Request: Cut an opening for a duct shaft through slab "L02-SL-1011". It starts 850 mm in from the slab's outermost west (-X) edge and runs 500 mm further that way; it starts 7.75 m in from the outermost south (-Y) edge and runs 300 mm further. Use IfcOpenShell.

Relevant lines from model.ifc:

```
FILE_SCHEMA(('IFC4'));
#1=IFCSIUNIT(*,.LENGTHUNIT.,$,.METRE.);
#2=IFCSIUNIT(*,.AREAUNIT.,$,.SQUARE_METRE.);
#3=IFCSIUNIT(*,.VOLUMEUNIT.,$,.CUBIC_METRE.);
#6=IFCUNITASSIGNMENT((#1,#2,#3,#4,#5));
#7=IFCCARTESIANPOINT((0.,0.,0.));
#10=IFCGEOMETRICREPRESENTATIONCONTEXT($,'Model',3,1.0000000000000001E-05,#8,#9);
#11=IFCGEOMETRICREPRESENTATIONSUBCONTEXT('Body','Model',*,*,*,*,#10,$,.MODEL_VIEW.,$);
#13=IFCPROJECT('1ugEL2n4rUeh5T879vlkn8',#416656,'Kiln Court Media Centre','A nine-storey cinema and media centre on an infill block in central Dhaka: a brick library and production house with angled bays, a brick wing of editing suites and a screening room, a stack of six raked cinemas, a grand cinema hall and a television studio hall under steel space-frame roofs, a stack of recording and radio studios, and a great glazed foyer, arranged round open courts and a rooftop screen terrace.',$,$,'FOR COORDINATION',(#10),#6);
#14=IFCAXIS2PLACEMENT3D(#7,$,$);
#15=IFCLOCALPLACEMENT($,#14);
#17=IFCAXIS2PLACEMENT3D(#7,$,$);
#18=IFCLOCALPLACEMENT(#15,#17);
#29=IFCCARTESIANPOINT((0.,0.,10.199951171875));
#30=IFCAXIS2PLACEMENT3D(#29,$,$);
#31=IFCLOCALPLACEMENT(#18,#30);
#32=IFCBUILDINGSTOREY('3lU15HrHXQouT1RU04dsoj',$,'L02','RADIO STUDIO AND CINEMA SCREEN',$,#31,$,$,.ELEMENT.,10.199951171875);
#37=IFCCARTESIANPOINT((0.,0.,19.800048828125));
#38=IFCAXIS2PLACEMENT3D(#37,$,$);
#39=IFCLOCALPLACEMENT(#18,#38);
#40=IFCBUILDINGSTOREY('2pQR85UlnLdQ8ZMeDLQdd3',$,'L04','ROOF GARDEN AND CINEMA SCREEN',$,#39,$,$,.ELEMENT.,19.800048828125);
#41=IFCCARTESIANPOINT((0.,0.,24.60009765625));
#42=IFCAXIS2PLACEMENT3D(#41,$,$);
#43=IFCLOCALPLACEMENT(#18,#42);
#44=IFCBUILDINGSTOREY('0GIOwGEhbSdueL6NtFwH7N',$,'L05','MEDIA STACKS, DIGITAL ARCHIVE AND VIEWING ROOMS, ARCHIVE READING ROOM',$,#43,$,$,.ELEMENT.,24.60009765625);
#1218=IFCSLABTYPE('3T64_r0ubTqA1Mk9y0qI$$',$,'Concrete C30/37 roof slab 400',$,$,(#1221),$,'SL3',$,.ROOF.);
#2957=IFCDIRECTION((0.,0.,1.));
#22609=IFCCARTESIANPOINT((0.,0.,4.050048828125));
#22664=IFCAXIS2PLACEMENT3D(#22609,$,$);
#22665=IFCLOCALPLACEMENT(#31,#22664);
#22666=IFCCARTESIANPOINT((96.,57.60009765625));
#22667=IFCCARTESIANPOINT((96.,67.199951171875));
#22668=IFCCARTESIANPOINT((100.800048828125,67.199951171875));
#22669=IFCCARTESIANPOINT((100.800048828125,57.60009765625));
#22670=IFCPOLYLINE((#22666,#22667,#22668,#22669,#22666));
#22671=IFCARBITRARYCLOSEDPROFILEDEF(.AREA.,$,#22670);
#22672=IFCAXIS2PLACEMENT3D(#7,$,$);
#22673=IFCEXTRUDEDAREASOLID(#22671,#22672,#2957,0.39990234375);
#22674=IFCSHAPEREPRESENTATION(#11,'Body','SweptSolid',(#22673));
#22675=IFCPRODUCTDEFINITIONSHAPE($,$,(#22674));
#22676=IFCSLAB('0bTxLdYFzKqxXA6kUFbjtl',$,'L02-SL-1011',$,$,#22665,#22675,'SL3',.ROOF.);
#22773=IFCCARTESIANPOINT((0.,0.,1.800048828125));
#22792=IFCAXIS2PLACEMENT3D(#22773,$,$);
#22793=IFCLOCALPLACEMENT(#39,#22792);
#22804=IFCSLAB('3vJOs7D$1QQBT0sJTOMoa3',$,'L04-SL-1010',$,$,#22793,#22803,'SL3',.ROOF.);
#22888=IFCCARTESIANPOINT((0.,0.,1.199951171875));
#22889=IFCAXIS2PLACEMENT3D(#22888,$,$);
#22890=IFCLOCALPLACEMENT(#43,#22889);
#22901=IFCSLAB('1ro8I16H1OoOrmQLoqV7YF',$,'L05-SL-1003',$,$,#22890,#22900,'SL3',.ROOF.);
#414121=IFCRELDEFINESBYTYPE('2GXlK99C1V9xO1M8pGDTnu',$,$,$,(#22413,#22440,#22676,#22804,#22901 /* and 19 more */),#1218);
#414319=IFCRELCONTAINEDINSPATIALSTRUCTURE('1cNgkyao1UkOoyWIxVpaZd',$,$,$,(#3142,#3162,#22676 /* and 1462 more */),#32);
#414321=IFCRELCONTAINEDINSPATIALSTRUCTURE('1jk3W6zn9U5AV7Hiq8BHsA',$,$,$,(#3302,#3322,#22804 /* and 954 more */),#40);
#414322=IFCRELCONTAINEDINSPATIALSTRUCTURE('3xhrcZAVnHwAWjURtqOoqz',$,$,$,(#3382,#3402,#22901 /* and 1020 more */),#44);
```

```python
import numpy as np
import ifcopenshell
import ifcopenshell.api.feature
import ifcopenshell.api.geometry
import ifcopenshell.api.root
import ifcopenshell.geom
import ifcopenshell.util.placement
import ifcopenshell.util.representation
import ifcopenshell.util.shape
import ifcopenshell.util.unit

model = ifcopenshell.open("model.ifc")
unit_scale = ifcopenshell.util.unit.calculate_unit_scale(model)
settings = ifcopenshell.geom.settings()


def volume(element):
    """Net volume in cubic metres, openings subtracted."""
    shape = ifcopenshell.geom.create_shape(settings, element)
    return ifcopenshell.util.shape.get_volume(shape.geometry)


slab = model.by_guid("0bTxLdYFzKqxXA6kUFbjtl")
before = volume(slab)

# Extent in the slab's own axes, in metres. The edges named are its -X and -Y sides.
slab_shape = ifcopenshell.geom.create_shape(settings, slab)
vertices = ifcopenshell.util.shape.get_vertices(slab_shape.geometry)
x_min, y_min, bottom = vertices.min(axis=0)
top = vertices[:, 2].max()

opening = ifcopenshell.api.root.create_entity(model, ifc_class="IfcOpeningElement", name="Duct shaft opening", predefined_type="OPENING")
context = ifcopenshell.util.representation.get_context(model, "Model", "Body", "MODEL_VIEW")
width, depth = 0.5, 0.3
outline = [(0.0, 0.0), (width, 0.0), (width, depth), (0.0, depth), (0.0, 0.0)]
# Overshoot both faces by 50 mm so the cut is clean.
shape = ifcopenshell.api.geometry.add_slab_representation(
    model, context=context, depth=top - bottom + 0.1, polyline=outline
)
ifcopenshell.api.geometry.assign_representation(model, product=opening, representation=shape)

matrix = ifcopenshell.util.placement.get_local_placement(slab.ObjectPlacement)
matrix[:, 3] = matrix @ np.append(np.array([x_min + 0.85, y_min + 7.75, bottom - 0.05]) / unit_scale, 1.0)
ifcopenshell.api.geometry.edit_object_placement(model, product=opening, matrix=matrix, is_si=False)
ifcopenshell.api.feature.add_feature(model, feature=opening, element=slab)

after = volume(slab)

print(f"slab volume {before:.3f} -> {after:.3f} m3")

model.write("model_edited.ifc")
```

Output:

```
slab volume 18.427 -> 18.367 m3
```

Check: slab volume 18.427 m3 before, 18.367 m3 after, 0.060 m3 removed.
